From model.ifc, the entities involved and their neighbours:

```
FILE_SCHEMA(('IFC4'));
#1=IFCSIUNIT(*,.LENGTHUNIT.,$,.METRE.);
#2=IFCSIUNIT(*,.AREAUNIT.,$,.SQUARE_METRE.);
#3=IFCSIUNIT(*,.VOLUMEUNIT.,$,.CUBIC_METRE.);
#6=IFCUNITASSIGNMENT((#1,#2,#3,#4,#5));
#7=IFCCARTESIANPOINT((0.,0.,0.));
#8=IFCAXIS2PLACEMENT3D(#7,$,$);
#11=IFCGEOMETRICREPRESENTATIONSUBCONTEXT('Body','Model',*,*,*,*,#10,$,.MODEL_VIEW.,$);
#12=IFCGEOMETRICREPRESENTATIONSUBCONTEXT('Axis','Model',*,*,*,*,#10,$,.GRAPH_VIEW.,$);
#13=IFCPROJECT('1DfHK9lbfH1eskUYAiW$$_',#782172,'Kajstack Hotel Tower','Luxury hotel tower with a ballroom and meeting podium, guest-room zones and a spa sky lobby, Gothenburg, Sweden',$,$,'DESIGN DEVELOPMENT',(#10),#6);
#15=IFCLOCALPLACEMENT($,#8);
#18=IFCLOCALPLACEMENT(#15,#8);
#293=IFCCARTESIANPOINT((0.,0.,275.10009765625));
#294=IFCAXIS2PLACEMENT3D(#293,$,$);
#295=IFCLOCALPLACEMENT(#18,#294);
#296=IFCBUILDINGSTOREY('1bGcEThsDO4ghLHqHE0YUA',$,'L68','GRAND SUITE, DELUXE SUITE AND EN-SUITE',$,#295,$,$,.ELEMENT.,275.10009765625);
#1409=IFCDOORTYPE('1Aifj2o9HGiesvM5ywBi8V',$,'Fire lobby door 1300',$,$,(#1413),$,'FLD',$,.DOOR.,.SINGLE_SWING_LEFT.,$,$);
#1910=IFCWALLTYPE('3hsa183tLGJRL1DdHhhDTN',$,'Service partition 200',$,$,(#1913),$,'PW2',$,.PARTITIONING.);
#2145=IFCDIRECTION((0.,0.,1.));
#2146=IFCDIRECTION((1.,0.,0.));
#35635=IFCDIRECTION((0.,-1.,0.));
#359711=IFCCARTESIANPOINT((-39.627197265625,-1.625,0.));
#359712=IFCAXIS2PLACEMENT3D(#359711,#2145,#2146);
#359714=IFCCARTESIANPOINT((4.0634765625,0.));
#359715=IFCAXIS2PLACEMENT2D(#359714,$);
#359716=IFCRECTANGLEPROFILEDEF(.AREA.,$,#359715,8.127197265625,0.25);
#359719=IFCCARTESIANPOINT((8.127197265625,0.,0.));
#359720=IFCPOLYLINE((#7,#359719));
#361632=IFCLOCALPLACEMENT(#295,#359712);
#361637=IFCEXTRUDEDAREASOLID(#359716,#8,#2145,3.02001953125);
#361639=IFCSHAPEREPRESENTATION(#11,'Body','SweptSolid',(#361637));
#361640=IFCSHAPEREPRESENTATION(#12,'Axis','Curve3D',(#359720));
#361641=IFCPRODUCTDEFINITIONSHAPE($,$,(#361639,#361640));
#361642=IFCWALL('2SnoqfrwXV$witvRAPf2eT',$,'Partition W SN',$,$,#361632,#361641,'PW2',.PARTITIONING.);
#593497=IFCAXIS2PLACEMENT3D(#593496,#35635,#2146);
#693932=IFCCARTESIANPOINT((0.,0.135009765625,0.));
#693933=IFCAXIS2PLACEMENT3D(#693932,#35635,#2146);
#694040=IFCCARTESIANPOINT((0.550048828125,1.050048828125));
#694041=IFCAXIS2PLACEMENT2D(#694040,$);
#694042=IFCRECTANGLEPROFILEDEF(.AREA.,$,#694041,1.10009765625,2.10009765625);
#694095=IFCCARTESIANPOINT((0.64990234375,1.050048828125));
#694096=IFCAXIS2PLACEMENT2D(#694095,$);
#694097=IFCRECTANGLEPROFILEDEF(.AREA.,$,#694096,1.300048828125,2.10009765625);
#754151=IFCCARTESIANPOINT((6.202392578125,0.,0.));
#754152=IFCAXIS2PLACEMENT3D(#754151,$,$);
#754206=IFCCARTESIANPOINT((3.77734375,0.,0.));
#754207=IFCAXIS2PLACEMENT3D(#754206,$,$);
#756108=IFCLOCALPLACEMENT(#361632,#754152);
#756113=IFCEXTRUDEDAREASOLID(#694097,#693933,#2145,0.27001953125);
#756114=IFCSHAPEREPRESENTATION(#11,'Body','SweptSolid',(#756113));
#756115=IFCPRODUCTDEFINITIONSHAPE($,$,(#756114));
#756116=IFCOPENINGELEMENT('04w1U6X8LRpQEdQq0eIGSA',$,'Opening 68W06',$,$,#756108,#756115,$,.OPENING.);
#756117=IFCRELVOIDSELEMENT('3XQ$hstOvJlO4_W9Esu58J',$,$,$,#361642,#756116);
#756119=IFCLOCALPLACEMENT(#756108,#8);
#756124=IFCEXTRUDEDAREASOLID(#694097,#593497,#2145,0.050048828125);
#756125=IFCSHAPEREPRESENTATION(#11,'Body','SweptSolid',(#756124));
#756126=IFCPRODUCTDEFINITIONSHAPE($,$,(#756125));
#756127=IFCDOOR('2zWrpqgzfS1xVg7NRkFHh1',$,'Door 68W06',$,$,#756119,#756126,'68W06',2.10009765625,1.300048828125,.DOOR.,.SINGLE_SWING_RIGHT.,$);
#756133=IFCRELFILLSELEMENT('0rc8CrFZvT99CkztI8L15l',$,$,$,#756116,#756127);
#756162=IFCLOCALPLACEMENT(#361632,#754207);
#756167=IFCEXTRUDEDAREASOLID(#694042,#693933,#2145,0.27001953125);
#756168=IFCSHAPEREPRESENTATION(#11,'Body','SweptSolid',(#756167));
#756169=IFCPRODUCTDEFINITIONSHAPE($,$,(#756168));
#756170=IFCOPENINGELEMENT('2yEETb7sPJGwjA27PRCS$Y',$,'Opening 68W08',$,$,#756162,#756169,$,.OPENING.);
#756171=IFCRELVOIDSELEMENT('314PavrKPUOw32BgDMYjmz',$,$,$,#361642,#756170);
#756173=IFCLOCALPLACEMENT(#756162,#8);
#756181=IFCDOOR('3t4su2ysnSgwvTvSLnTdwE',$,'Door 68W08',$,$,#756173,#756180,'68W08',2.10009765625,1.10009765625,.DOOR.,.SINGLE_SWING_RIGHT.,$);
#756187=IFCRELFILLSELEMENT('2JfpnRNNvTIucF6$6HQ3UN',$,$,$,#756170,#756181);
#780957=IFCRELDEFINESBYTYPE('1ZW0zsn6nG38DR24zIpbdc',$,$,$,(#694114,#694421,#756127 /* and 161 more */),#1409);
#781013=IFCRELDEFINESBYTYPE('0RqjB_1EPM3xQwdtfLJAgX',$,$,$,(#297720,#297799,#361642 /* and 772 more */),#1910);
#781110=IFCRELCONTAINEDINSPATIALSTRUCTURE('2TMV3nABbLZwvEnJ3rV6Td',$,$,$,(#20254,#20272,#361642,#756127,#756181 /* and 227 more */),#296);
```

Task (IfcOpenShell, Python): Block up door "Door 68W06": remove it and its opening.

```python
import ifcopenshell
import ifcopenshell.api.feature
import ifcopenshell.api.root
import ifcopenshell.geom
import ifcopenshell.util.shape

model = ifcopenshell.open("model.ifc")
settings = ifcopenshell.geom.settings()


def volume(element):
    """Net volume in cubic metres, openings subtracted."""
    shape = ifcopenshell.geom.create_shape(settings, element)
    return ifcopenshell.util.shape.get_volume(shape.geometry)


door = model.by_guid("2zWrpqgzfS1xVg7NRkFHh1")
opening = door.FillsVoids[0].RelatingOpeningElement
wall = opening.VoidsElements[0].RelatingBuildingElement
before = volume(wall)

ifcopenshell.api.root.remove_product(model, product=door)
ifcopenshell.api.feature.remove_feature(model, feature=opening)

after = volume(wall)

print(f"wall volume {before:.3f} -> {after:.3f} m3")

model.write("model_rev.ifc")
```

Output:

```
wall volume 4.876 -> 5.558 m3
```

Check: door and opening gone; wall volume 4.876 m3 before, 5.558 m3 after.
